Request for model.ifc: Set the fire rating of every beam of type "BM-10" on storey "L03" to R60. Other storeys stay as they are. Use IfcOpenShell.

First a look at what the model holds.

```python
import ifcopenshell
import ifcopenshell.util.element

model = ifcopenshell.open("model.ifc")
print(model.schema)
storey = next(s for s in model.by_type("IfcBuildingStorey") if s.Name == "L03")
beams = [e for e in ifcopenshell.util.element.get_decomposition(storey) if e.is_a("IfcBeam")]
seen = {}
for e in beams:
    element_type = ifcopenshell.util.element.get_type(e)
    key = (element_type.Name if element_type != e and element_type else None, ifcopenshell.util.element.get_pset(e, "Pset_BeamCommon", "FireRating"))
    seen[key] = seen.get(key, 0) + 1
for (name, value), count in sorted(seen.items(), key=str):
    print(count, "x", name, "|", value)
```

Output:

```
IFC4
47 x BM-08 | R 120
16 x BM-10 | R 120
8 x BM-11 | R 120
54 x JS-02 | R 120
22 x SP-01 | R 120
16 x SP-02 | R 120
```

```python
import ifcopenshell
import ifcopenshell.api.pset
import ifcopenshell.util.element

model = ifcopenshell.open("model.ifc")

storey = next(s for s in model.by_type("IfcBuildingStorey") if s.Name == "L03")
beams = [e for e in ifcopenshell.util.element.get_decomposition(storey) if e.is_a("IfcBeam")]

count = 0
for e in beams:
    element_type = ifcopenshell.util.element.get_type(e)
    if element_type in (None, e) or element_type.Name != "BM-10":
        continue
    # add_pset returns the element's existing set when there is one.
    pset = ifcopenshell.api.pset.add_pset(model, product=e, name="Pset_BeamCommon")
    ifcopenshell.api.pset.edit_pset(model, pset=pset, properties={"FireRating": "R60"})
    count += 1

print(count, "beams updated")

model.write("model_edited.ifc")
```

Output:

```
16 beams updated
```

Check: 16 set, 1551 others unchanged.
